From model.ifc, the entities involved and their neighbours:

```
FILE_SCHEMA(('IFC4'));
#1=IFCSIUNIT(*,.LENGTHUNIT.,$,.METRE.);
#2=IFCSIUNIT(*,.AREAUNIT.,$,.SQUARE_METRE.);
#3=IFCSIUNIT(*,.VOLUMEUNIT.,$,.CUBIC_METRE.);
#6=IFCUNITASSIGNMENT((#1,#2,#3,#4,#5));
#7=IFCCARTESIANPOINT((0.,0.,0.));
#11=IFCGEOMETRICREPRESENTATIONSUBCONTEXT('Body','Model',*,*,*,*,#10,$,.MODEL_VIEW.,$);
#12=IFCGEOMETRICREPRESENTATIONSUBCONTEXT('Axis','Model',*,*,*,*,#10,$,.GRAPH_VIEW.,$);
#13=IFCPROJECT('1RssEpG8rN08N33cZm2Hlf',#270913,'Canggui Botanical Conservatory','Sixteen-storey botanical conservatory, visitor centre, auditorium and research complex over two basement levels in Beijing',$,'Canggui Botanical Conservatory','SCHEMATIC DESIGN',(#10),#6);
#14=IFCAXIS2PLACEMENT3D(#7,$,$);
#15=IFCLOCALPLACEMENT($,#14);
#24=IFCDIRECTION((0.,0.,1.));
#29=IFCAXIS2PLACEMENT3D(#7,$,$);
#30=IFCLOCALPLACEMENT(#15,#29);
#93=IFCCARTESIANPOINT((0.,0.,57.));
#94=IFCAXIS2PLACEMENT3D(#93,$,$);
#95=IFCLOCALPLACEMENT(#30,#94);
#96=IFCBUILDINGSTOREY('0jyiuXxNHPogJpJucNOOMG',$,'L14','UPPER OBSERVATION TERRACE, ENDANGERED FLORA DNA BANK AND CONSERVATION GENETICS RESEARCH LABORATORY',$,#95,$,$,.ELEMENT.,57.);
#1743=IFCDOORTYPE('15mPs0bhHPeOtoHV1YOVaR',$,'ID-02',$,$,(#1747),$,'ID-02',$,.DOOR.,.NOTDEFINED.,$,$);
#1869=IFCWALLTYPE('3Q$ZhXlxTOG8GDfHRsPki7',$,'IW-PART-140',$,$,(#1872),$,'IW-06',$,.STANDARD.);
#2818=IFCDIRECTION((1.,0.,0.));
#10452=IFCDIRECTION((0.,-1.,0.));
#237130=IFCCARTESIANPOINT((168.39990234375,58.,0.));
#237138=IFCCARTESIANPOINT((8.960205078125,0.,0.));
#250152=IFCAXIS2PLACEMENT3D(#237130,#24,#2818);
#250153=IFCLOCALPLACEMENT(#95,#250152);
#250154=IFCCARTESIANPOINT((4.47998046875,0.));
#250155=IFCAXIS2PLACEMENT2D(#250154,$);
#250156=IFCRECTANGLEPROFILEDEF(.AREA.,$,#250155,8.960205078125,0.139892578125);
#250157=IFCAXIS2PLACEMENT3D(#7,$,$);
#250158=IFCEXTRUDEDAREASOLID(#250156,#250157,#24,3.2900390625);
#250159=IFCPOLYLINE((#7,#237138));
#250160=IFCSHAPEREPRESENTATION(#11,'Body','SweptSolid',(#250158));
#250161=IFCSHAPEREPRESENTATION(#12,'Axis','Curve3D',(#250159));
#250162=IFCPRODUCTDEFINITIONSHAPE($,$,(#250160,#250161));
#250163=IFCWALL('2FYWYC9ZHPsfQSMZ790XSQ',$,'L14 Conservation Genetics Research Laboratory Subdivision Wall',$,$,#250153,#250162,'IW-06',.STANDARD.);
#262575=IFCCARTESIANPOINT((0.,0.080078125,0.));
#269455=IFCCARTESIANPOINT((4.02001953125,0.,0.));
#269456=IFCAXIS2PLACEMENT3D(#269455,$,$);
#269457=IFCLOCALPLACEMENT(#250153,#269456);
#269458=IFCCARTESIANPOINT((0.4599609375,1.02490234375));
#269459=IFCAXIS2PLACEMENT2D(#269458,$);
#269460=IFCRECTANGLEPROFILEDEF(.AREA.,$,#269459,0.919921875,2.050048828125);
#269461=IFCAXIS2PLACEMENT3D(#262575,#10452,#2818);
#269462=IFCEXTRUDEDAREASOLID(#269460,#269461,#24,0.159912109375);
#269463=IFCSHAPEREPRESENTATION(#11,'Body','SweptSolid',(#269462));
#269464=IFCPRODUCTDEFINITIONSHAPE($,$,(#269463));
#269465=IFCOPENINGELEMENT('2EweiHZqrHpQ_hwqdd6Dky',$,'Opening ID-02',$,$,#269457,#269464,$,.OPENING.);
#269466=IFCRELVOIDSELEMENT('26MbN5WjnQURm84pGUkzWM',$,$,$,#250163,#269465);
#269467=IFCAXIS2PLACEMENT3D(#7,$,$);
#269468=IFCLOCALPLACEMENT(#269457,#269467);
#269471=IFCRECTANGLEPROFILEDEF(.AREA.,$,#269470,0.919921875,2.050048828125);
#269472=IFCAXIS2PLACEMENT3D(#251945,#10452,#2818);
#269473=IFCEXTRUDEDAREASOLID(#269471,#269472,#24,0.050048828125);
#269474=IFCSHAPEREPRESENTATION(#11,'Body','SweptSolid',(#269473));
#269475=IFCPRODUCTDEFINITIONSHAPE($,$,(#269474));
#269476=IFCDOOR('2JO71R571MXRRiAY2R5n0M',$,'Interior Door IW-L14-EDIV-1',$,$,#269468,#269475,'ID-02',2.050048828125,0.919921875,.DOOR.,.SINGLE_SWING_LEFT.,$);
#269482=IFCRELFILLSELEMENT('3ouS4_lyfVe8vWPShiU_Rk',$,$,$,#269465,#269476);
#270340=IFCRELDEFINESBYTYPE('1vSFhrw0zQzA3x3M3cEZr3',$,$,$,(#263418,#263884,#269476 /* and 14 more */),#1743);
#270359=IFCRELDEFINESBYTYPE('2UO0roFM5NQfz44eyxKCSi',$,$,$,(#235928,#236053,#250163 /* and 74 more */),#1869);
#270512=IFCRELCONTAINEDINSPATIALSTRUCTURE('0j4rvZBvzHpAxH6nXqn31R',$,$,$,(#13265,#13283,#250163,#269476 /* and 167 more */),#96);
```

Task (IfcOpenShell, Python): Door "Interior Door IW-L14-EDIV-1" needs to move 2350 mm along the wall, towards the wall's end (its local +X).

```python
import ifcopenshell
import ifcopenshell.api.geometry
import ifcopenshell.util.placement

model = ifcopenshell.open("model.ifc")

door = model.by_guid("2JO71R571MXRRiAY2R5n0M")
opening = door.FillsVoids[0].RelatingOpeningElement
wall = opening.VoidsElements[0].RelatingBuildingElement

wall_matrix = ifcopenshell.util.placement.get_local_placement(wall.ObjectPlacement)
shift = wall_matrix[:3, 0] * 2.35
before = ifcopenshell.util.placement.get_local_placement(door.ObjectPlacement)[:3, 3].copy()

# The door is placed relative to its opening, so it follows when the opening moves.
matrix = ifcopenshell.util.placement.get_local_placement(opening.ObjectPlacement)
matrix[:3, 3] += shift
ifcopenshell.api.geometry.edit_object_placement(
    model, product=opening, matrix=matrix, is_si=False, should_transform_children=True
)

after = ifcopenshell.util.placement.get_local_placement(door.ObjectPlacement)[:3, 3]
print("door moved by", (after - before).round(3) + 0.0)

model.write("model_edited.ifc")
```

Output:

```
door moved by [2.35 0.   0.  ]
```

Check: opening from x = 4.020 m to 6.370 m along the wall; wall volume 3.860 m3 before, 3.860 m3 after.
